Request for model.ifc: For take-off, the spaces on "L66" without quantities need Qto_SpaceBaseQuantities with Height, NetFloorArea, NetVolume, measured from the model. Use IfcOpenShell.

First a look at what the model holds.

```python
import ifcopenshell
import ifcopenshell.util.element
import ifcopenshell.util.unit

model = ifcopenshell.open("model.ifc")
print(model.schema)
for unit_type in ("LENGTHUNIT", "AREAUNIT", "VOLUMEUNIT"):
    print(unit_type, ifcopenshell.util.unit.calculate_unit_scale(model, unit_type))
storey = next(s for s in model.by_type("IfcBuildingStorey") if s.Name == "L66")
spaces = [e for e in ifcopenshell.util.element.get_decomposition(storey) if e.is_a("IfcSpace")]
for e in sorted(spaces, key=lambda e: e.id()):
    print(e.id(), e.is_a(), e.Name, list(ifcopenshell.util.element.get_psets(e, qtos_only=True)), sep=" | ")
```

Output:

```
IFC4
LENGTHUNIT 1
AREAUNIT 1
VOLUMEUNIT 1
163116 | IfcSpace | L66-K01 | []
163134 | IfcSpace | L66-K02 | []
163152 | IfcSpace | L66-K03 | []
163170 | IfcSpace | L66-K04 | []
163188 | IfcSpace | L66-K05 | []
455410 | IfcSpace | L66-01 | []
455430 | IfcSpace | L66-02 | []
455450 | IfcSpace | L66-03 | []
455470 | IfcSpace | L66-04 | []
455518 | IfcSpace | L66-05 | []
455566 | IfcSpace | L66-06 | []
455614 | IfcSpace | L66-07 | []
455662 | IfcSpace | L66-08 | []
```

```python
import ifcopenshell
import ifcopenshell.api.pset
import ifcopenshell.geom
import ifcopenshell.util.element
import ifcopenshell.util.shape
import ifcopenshell.util.unit

model = ifcopenshell.open("model.ifc")
unit_scale = ifcopenshell.util.unit.calculate_unit_scale(model)
area_scale = ifcopenshell.util.unit.calculate_unit_scale(model, "AREAUNIT")
volume_scale = ifcopenshell.util.unit.calculate_unit_scale(model, "VOLUMEUNIT")
settings = ifcopenshell.geom.settings()

storey = next(s for s in model.by_type("IfcBuildingStorey") if s.Name == "L66")
spaces = [e for e in ifcopenshell.util.element.get_decomposition(storey) if e.is_a("IfcSpace")]

for e in sorted(spaces, key=lambda e: e.id()):
    if ifcopenshell.util.element.get_psets(e, qtos_only=True, should_inherit=False):
        continue
    # Geometry comes back in metres, in the element's own axes.
    shape = ifcopenshell.geom.create_shape(settings, e)
    values = {
        "Height": ifcopenshell.util.shape.get_z(shape.geometry) / unit_scale,
        "NetFloorArea": ifcopenshell.util.shape.get_footprint_area(shape.geometry) / area_scale,
        "NetVolume": ifcopenshell.util.shape.get_volume(shape.geometry) / volume_scale,
    }
    qto = ifcopenshell.api.pset.add_qto(model, product=e, name="Qto_SpaceBaseQuantities")
    ifcopenshell.api.pset.edit_qto(model, qto=qto, properties=values)
    print(e.id(), {k: round(v, 3) for k, v in values.items()})

model.write("model_edited.ifc")
```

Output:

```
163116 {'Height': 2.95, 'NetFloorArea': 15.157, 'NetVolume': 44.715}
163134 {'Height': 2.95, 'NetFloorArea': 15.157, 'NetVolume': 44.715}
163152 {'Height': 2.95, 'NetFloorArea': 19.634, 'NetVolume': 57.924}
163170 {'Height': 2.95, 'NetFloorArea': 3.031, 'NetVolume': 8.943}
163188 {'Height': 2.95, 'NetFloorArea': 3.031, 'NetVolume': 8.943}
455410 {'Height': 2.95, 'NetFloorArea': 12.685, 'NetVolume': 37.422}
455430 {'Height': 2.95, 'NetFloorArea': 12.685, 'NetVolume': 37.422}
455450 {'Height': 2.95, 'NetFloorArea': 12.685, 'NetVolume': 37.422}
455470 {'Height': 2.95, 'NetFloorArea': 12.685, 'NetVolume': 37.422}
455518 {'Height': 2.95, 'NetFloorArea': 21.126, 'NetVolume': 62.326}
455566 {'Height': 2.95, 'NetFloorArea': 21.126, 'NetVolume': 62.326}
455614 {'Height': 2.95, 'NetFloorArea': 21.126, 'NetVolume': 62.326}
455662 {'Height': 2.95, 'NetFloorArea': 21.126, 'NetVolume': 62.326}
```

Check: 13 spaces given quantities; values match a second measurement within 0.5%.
